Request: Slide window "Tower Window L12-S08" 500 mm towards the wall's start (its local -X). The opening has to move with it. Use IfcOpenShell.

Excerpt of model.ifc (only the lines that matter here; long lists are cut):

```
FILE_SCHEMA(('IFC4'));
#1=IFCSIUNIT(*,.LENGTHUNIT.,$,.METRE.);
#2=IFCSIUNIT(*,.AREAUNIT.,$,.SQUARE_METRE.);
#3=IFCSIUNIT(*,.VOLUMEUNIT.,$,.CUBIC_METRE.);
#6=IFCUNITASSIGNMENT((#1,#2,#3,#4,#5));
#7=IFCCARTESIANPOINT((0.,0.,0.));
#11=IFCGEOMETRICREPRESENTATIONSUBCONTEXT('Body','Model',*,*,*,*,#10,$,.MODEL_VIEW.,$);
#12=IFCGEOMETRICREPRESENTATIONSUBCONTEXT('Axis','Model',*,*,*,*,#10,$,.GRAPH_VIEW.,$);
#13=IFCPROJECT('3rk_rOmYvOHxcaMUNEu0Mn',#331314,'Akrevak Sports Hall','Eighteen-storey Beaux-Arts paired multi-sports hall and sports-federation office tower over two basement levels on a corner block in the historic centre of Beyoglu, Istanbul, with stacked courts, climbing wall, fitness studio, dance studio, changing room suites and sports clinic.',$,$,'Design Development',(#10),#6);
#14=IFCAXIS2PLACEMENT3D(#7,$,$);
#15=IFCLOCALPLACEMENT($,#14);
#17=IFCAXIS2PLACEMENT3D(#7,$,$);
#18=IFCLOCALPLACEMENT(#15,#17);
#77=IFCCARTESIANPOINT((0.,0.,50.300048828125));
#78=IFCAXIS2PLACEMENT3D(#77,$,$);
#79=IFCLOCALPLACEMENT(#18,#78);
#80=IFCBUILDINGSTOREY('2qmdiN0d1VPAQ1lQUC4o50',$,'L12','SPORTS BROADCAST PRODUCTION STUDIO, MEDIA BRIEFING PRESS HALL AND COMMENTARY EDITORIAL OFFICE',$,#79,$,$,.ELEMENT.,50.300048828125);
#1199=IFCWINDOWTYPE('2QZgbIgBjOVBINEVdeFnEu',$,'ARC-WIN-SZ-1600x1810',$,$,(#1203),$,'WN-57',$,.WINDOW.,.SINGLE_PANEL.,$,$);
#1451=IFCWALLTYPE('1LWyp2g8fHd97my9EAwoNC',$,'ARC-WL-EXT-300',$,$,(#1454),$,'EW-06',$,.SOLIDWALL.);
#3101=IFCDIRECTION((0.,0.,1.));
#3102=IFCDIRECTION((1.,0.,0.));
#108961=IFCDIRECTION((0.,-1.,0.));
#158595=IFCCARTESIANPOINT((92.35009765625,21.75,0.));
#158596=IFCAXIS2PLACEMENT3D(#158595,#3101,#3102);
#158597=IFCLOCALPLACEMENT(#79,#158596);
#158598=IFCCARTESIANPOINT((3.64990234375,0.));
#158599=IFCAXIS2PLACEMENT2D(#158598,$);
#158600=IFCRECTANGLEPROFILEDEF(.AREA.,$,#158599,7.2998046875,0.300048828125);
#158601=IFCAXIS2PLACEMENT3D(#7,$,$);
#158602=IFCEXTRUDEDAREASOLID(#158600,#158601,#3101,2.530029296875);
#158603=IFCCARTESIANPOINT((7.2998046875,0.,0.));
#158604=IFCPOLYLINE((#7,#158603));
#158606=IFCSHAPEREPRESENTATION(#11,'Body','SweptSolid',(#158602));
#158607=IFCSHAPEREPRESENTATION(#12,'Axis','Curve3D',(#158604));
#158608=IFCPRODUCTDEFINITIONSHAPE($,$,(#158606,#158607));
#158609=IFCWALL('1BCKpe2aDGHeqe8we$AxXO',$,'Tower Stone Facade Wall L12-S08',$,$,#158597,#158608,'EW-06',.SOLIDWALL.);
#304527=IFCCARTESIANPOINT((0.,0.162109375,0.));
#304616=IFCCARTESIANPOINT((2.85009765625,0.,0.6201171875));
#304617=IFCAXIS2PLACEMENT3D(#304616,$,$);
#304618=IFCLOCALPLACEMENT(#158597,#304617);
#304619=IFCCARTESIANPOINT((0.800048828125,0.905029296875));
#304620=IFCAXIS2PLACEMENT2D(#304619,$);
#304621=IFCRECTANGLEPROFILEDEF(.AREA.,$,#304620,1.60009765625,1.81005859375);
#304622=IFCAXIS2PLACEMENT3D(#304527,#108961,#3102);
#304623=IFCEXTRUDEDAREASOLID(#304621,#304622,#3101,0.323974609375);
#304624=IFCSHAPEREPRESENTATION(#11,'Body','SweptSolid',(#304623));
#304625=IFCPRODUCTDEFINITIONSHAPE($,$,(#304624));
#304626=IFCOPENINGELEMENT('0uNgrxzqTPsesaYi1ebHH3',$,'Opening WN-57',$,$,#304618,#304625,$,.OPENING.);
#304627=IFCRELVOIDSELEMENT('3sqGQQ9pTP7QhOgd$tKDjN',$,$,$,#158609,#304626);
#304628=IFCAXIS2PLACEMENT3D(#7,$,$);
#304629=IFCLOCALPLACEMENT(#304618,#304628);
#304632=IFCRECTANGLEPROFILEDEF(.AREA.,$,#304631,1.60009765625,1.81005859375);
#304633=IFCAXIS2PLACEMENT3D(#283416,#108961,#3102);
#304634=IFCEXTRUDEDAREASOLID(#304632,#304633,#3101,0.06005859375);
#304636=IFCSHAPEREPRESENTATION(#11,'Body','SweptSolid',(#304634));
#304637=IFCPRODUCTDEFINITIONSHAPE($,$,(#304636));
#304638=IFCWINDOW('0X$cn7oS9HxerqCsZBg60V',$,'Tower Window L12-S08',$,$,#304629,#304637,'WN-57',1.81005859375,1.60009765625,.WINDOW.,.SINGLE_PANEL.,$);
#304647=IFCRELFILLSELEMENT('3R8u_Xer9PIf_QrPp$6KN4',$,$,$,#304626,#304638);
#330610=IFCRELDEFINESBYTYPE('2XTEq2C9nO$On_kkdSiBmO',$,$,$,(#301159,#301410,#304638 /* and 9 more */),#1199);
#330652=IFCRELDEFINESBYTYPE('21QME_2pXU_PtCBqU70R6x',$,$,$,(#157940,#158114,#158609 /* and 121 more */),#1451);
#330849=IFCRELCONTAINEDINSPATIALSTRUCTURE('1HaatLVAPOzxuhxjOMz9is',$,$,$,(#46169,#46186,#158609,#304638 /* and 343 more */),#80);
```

```python
import ifcopenshell
import ifcopenshell.api.geometry
import ifcopenshell.util.placement
import ifcopenshell.util.unit

model = ifcopenshell.open("model.ifc")
unit_scale = ifcopenshell.util.unit.calculate_unit_scale(model)

window = model.by_id(304638)
opening = window.FillsVoids[0].RelatingOpeningElement
wall = opening.VoidsElements[0].RelatingBuildingElement

wall_matrix = ifcopenshell.util.placement.get_local_placement(wall.ObjectPlacement)
shift = wall_matrix[:3, 0] * -0.5 / unit_scale
before = ifcopenshell.util.placement.get_local_placement(window.ObjectPlacement)[:3, 3].copy()

# The window is placed relative to its opening, so it follows when the opening moves.
matrix = ifcopenshell.util.placement.get_local_placement(opening.ObjectPlacement)
matrix[:3, 3] += shift
ifcopenshell.api.geometry.edit_object_placement(
    model, product=opening, matrix=matrix, is_si=False, should_transform_children=True
)

after = ifcopenshell.util.placement.get_local_placement(window.ObjectPlacement)[:3, 3]
print("window moved by", (after - before).round(3) + 0.0)

model.write("model_v2.ifc")
```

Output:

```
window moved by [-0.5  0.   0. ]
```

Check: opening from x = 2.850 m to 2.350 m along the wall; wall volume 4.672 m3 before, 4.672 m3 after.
